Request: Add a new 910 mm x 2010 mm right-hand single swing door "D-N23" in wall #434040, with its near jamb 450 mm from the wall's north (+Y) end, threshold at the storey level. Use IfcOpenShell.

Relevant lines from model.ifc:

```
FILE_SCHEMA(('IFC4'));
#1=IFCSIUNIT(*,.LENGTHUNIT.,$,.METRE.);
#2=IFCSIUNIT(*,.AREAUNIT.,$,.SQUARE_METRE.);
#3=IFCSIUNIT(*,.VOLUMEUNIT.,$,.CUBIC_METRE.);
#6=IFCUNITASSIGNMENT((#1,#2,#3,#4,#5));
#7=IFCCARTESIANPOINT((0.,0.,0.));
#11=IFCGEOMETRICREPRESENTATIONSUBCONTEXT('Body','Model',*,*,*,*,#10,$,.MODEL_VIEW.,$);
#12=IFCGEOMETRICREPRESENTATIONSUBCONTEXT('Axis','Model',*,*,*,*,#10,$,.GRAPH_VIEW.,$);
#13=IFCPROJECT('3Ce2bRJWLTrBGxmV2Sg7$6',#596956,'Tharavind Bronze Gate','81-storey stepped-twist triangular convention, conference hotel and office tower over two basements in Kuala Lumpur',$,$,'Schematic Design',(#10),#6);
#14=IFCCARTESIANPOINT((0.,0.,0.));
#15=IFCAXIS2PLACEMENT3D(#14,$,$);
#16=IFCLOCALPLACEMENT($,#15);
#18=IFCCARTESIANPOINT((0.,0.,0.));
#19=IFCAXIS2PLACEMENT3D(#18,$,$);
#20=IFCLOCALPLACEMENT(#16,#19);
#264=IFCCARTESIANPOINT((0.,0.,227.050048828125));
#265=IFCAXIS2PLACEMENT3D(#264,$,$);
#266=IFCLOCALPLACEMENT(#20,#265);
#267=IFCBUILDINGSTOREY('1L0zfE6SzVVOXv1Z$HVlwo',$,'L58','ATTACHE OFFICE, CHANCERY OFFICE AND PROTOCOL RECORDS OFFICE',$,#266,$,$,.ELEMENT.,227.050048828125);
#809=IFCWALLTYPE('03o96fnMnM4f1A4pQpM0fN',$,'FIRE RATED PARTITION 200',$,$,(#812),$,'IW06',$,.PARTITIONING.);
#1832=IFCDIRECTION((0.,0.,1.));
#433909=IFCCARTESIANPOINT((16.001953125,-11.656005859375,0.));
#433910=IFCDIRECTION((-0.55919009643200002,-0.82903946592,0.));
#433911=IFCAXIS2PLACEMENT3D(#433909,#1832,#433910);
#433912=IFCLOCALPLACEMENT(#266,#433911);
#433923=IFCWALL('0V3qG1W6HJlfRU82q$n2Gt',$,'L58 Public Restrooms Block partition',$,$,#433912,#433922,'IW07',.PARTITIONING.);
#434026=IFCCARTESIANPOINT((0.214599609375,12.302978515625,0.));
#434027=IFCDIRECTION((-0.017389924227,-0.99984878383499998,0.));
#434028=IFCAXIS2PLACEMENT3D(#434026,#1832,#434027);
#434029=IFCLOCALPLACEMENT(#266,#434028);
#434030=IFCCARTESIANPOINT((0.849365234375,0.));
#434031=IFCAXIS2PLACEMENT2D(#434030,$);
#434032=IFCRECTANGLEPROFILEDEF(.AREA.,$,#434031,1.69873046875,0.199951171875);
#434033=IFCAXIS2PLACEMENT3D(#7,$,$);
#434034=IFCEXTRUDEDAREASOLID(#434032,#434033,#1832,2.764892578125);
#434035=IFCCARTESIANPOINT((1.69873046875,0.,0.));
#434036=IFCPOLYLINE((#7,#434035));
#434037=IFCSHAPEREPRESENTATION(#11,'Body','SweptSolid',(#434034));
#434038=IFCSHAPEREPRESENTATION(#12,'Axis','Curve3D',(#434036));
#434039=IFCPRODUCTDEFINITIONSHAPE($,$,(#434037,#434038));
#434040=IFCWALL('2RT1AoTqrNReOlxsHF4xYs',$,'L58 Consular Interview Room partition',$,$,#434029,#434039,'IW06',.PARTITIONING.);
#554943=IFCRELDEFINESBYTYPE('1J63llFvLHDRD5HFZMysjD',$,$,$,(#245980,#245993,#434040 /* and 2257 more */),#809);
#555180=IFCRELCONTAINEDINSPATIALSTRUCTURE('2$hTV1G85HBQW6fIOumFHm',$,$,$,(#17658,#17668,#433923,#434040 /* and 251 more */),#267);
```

```python
import numpy as np
import ifcopenshell
import ifcopenshell.api.feature
import ifcopenshell.api.geometry
import ifcopenshell.api.root
import ifcopenshell.api.spatial
import ifcopenshell.geom
import ifcopenshell.util.element
import ifcopenshell.util.placement
import ifcopenshell.util.representation
import ifcopenshell.util.shape
import ifcopenshell.util.unit

model = ifcopenshell.open("model.ifc")
unit_scale = ifcopenshell.util.unit.calculate_unit_scale(model)
settings = ifcopenshell.geom.settings()


def volume(element):
    """Net volume in cubic metres, openings subtracted."""
    shape = ifcopenshell.geom.create_shape(settings, element)
    return ifcopenshell.util.shape.get_volume(shape.geometry)


wall = model.by_guid("2RT1AoTqrNReOlxsHF4xYs")
storey = ifcopenshell.util.element.get_container(wall, ifc_class="IfcBuildingStorey")
context = ifcopenshell.util.representation.get_context(model, "Model", "Body", "MODEL_VIEW")
before = volume(wall)

width, height, from_end, sill = 0.91, 2.01, 0.45, 0.0  # metres

# The wall runs along its own X axis, and the end named is its -X end.
wall_shape = ifcopenshell.geom.create_shape(settings, wall)
x, y, z = ifcopenshell.util.shape.get_vertices(wall_shape.geometry).T
start = x.min() + from_end
face, thickness = float(y.min()), float(y.max() - y.min())
wall_matrix = ifcopenshell.util.placement.get_local_placement(wall.ObjectPlacement)
level = ifcopenshell.util.placement.get_local_placement(storey.ObjectPlacement)[2, 3]


def in_wall(x, y):
    """Placement at x, y metres in the wall's axes, at sill height."""
    matrix = wall_matrix.copy()
    matrix[:, 3] = wall_matrix @ np.array([x / unit_scale, y / unit_scale, 0.0, 1.0])
    matrix[2, 3] = level + sill / unit_scale
    return matrix


# Opening: a box that overshoots both wall faces by 50 mm.
opening = ifcopenshell.api.root.create_entity(model, ifc_class="IfcOpeningElement", predefined_type="OPENING")
box = ifcopenshell.api.geometry.add_wall_representation(
    model, context=context, length=width, height=height, thickness=thickness + 0.1
)
ifcopenshell.api.geometry.assign_representation(model, product=opening, representation=box)
ifcopenshell.api.geometry.edit_object_placement(model, product=opening, matrix=in_wall(start, face - 0.05), is_si=False)
ifcopenshell.api.feature.add_feature(model, feature=opening, element=wall)

door = ifcopenshell.api.root.create_entity(model, ifc_class="IfcDoor", name="D-N23", predefined_type="DOOR")
door.OverallWidth, door.OverallHeight = width / unit_scale, height / unit_scale
door.OperationType = "SINGLE_SWING_RIGHT"
body = ifcopenshell.api.geometry.add_door_representation(
    model,
    context=context,
    overall_width=door.OverallWidth,
    overall_height=door.OverallHeight,
    operation_type="SINGLE_SWING_RIGHT",
    lining_properties={"LiningDepth": thickness / unit_scale, "ThresholdDepth": thickness / unit_scale},
)
ifcopenshell.api.geometry.assign_representation(model, product=door, representation=body)
ifcopenshell.api.spatial.assign_container(model, products=[door], relating_structure=storey)
ifcopenshell.api.feature.add_filling(model, opening=opening, element=door)

# The lining spans the wall, so the door starts at the wall face.
ifcopenshell.api.geometry.edit_object_placement(model, product=door, matrix=in_wall(start, face), is_si=False)

after = volume(wall)

print(f"wall volume {before:.3f} -> {after:.3f} m3")

model.write("model_v2.ifc")
```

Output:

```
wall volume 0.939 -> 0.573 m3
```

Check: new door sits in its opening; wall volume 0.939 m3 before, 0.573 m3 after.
